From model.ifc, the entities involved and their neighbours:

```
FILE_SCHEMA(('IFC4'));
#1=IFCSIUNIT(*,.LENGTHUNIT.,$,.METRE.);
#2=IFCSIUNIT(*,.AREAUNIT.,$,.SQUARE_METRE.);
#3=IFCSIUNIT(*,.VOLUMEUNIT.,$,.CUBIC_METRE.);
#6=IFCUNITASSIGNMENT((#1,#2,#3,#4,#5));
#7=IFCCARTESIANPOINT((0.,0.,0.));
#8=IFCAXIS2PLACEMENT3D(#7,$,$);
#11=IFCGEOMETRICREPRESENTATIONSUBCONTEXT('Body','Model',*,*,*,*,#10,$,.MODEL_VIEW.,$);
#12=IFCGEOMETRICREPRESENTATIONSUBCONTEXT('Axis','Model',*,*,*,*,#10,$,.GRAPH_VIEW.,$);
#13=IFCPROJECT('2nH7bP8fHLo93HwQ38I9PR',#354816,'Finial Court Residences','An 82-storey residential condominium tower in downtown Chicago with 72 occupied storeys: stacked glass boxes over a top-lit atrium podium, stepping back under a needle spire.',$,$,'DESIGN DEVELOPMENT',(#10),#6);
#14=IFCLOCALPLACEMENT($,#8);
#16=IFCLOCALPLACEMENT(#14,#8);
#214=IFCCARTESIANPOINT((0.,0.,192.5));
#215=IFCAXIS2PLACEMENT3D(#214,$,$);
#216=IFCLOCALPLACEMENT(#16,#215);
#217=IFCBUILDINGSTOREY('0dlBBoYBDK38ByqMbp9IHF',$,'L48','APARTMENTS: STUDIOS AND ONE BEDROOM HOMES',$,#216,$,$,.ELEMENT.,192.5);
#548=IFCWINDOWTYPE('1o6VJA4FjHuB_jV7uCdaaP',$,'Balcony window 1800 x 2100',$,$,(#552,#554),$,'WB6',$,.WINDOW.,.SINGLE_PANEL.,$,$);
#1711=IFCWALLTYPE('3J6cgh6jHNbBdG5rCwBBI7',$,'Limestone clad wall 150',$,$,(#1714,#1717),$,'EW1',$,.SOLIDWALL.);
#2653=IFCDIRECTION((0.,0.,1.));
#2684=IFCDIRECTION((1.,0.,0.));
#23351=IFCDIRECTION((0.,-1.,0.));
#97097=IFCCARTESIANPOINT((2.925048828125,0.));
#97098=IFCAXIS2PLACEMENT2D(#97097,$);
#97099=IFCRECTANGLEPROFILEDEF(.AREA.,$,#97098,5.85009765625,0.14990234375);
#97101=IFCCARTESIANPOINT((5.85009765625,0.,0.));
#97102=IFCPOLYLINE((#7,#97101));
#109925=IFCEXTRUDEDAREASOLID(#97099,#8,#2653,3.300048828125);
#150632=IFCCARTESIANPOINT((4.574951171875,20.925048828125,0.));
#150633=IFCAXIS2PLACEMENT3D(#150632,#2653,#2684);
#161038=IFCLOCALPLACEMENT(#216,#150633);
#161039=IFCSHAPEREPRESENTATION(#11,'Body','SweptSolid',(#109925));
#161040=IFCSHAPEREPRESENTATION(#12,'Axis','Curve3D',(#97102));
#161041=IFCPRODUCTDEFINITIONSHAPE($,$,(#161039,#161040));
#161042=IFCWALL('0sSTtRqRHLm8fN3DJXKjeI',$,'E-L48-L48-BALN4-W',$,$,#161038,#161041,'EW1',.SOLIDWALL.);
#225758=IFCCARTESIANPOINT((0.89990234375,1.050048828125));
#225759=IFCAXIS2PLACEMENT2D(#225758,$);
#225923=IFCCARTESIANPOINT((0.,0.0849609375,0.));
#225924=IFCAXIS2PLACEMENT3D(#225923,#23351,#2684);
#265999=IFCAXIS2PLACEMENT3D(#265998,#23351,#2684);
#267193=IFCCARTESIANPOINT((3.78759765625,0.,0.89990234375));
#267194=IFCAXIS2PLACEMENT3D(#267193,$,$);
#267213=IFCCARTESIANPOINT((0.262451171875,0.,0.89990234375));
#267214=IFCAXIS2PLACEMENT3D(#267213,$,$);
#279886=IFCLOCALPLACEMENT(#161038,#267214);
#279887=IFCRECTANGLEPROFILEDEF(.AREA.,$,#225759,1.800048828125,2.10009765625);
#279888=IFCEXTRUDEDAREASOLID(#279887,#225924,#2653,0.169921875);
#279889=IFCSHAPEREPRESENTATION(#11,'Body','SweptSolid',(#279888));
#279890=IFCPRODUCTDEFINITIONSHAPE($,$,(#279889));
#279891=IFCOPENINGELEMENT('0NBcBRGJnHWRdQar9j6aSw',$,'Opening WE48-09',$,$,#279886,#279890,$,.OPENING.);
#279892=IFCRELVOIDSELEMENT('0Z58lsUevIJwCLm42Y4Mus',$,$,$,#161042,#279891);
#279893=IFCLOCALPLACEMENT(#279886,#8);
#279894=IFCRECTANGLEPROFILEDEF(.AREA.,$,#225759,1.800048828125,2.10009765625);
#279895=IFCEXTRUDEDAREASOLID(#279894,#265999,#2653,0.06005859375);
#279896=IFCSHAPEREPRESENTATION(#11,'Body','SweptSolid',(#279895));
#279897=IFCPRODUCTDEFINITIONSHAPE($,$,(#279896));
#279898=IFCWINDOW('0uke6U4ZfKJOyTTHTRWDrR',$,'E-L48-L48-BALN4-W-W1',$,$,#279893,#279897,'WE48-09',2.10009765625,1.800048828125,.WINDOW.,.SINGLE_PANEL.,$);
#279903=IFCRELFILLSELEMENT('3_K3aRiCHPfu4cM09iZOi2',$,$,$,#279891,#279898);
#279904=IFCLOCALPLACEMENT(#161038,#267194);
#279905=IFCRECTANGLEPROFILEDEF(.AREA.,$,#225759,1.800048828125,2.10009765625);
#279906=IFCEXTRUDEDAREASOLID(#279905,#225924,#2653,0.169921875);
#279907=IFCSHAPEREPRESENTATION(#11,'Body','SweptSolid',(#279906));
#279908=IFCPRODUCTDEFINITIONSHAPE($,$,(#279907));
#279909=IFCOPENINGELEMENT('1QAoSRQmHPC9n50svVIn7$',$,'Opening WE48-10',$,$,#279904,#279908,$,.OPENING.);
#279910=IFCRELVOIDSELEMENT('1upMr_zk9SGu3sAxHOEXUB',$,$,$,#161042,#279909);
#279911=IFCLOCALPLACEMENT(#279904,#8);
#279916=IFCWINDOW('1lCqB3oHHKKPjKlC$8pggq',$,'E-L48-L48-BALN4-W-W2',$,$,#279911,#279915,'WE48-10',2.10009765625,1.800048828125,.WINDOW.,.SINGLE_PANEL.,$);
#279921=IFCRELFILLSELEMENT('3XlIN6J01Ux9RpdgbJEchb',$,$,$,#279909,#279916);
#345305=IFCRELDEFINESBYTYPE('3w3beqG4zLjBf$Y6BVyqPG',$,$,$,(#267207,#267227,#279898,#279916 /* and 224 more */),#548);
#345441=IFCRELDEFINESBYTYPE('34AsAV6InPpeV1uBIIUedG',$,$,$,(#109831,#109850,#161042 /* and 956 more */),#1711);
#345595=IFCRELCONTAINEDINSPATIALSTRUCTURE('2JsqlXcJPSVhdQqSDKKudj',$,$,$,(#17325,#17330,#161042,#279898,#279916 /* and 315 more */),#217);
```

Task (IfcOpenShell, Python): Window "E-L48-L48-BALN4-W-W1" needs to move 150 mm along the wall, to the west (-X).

```python
import ifcopenshell
import ifcopenshell.api.geometry
import ifcopenshell.util.placement
import ifcopenshell.util.unit

model = ifcopenshell.open("model.ifc")
unit_scale = ifcopenshell.util.unit.calculate_unit_scale(model)

window = model.by_id(279898)
opening = window.FillsVoids[0].RelatingOpeningElement
wall = opening.VoidsElements[0].RelatingBuildingElement

wall_matrix = ifcopenshell.util.placement.get_local_placement(wall.ObjectPlacement)
shift = wall_matrix[:3, 0] * -0.15 / unit_scale
before = ifcopenshell.util.placement.get_local_placement(window.ObjectPlacement)[:3, 3].copy()

# The window is placed relative to its opening, so it follows when the opening moves.
matrix = ifcopenshell.util.placement.get_local_placement(opening.ObjectPlacement)
matrix[:3, 3] += shift
ifcopenshell.api.geometry.edit_object_placement(
    model, product=opening, matrix=matrix, is_si=False, should_transform_children=True
)

after = ifcopenshell.util.placement.get_local_placement(window.ObjectPlacement)[:3, 3]
print("window moved by", (after - before).round(3) + 0.0)

model.write("model_edited.ifc")
```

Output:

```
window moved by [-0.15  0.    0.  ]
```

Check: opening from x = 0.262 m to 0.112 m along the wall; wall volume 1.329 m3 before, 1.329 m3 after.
